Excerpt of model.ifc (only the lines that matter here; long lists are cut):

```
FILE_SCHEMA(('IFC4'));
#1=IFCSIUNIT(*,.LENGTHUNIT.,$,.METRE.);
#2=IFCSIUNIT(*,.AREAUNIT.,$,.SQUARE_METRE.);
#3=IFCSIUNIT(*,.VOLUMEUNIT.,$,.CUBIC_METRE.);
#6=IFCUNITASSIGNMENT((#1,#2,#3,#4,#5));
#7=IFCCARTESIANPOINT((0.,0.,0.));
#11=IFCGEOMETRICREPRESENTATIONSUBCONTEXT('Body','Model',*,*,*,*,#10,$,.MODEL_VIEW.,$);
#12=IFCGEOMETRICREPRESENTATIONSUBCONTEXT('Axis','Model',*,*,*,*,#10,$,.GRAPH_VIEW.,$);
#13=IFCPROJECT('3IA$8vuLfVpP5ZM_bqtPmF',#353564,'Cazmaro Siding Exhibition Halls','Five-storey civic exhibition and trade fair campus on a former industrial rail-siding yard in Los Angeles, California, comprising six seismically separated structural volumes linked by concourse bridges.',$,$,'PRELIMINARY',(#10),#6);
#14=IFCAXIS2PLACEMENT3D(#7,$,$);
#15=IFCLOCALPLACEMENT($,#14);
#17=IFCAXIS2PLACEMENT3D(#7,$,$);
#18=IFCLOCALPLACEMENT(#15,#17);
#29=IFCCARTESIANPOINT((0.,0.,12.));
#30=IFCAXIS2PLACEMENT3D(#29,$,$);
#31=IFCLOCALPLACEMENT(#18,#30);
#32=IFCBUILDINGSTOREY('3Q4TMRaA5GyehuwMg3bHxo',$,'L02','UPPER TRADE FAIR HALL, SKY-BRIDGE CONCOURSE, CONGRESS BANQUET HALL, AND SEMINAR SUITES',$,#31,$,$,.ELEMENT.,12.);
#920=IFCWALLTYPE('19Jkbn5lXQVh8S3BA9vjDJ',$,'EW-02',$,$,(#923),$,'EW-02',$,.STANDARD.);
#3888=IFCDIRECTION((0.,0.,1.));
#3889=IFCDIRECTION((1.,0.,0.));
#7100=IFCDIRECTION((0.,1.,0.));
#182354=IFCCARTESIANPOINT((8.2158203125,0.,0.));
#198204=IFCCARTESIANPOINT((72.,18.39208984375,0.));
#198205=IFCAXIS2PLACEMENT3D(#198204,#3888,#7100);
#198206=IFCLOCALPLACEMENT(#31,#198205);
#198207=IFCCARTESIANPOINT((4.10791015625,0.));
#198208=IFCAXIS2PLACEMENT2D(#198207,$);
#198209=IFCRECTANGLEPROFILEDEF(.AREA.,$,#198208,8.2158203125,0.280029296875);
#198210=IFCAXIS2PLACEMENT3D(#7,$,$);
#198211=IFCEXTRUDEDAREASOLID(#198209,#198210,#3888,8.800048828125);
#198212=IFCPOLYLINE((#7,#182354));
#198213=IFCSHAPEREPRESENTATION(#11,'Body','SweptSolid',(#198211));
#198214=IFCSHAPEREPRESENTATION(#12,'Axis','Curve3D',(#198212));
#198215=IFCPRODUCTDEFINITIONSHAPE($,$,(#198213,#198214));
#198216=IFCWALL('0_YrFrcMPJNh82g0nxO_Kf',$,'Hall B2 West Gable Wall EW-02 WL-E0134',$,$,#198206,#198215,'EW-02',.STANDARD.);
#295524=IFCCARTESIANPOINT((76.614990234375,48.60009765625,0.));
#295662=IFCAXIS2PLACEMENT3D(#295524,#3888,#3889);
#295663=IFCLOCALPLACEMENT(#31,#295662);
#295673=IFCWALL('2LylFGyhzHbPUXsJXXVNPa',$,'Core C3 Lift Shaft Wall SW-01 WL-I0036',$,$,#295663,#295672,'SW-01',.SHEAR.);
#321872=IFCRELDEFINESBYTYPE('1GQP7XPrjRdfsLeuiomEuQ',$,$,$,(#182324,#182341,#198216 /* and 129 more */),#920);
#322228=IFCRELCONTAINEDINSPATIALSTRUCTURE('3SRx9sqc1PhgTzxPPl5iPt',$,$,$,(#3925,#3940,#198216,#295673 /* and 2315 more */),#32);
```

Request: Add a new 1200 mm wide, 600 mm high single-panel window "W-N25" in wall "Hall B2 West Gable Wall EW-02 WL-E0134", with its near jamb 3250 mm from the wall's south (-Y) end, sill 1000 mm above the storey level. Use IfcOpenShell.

```python
import numpy as np
import ifcopenshell
import ifcopenshell.api.feature
import ifcopenshell.api.geometry
import ifcopenshell.api.root
import ifcopenshell.api.spatial
import ifcopenshell.geom
import ifcopenshell.util.element
import ifcopenshell.util.placement
import ifcopenshell.util.representation
import ifcopenshell.util.shape
import ifcopenshell.util.unit

model = ifcopenshell.open("model.ifc")
unit_scale = ifcopenshell.util.unit.calculate_unit_scale(model)
settings = ifcopenshell.geom.settings()


def volume(element):
    """Net volume in cubic metres, openings subtracted."""
    shape = ifcopenshell.geom.create_shape(settings, element)
    return ifcopenshell.util.shape.get_volume(shape.geometry)


wall = model.by_guid("0_YrFrcMPJNh82g0nxO_Kf")
storey = ifcopenshell.util.element.get_container(wall, ifc_class="IfcBuildingStorey")
context = ifcopenshell.util.representation.get_context(model, "Model", "Body", "MODEL_VIEW")
before = volume(wall)

width, height, from_end, sill = 1.2, 0.6, 3.25, 1  # metres

# The wall runs along its own X axis, and the end named is its -X end.
wall_shape = ifcopenshell.geom.create_shape(settings, wall)
x, y, z = ifcopenshell.util.shape.get_vertices(wall_shape.geometry).T
start = x.min() + from_end
face, thickness = float(y.min()), float(y.max() - y.min())
wall_matrix = ifcopenshell.util.placement.get_local_placement(wall.ObjectPlacement)
level = ifcopenshell.util.placement.get_local_placement(storey.ObjectPlacement)[2, 3]


def in_wall(x, y):
    """Placement at x, y metres in the wall's axes, at sill height."""
    matrix = wall_matrix.copy()
    matrix[:, 3] = wall_matrix @ np.array([x / unit_scale, y / unit_scale, 0.0, 1.0])
    matrix[2, 3] = level + sill / unit_scale
    return matrix


# Opening: a box that overshoots both wall faces by 50 mm.
opening = ifcopenshell.api.root.create_entity(model, ifc_class="IfcOpeningElement", predefined_type="OPENING")
box = ifcopenshell.api.geometry.add_wall_representation(
    model, context=context, length=width, height=height, thickness=thickness + 0.1
)
ifcopenshell.api.geometry.assign_representation(model, product=opening, representation=box)
ifcopenshell.api.geometry.edit_object_placement(model, product=opening, matrix=in_wall(start, face - 0.05), is_si=False)
ifcopenshell.api.feature.add_feature(model, feature=opening, element=wall)

window = ifcopenshell.api.root.create_entity(model, ifc_class="IfcWindow", name="W-N25", predefined_type="WINDOW")
window.OverallWidth, window.OverallHeight = width / unit_scale, height / unit_scale
window.PartitioningType = "SINGLE_PANEL"
body = ifcopenshell.api.geometry.add_window_representation(
    model,
    context=context,
    overall_width=window.OverallWidth,
    overall_height=window.OverallHeight,
    partition_type="SINGLE_PANEL",
)
ifcopenshell.api.geometry.assign_representation(model, product=window, representation=body)
ifcopenshell.api.spatial.assign_container(model, products=[window], relating_structure=storey)
ifcopenshell.api.feature.add_filling(model, opening=opening, element=window)

# Centre the window in the wall's thickness.
ifcopenshell.api.geometry.edit_object_placement(model, product=window, matrix=in_wall(start, face), is_si=False)
window_shape = ifcopenshell.geom.create_shape(settings, window)
depth = ifcopenshell.util.shape.get_vertices(window_shape.geometry)[:, 1]
offset = face + thickness / 2 - (depth.min() + depth.max()) / 2
ifcopenshell.api.geometry.edit_object_placement(model, product=window, matrix=in_wall(start, offset), is_si=False)

after = volume(wall)

print(f"wall volume {before:.3f} -> {after:.3f} m3")

model.write("model_updated.ifc")
```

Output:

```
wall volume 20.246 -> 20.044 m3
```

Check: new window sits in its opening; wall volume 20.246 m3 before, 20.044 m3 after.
